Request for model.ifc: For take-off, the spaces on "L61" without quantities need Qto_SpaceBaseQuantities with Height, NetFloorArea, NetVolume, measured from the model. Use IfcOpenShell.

First a look at what the model holds.

```python
import ifcopenshell
import ifcopenshell.util.element
import ifcopenshell.util.unit

model = ifcopenshell.open("model.ifc")
print(model.schema)
for unit_type in ("LENGTHUNIT", "AREAUNIT", "VOLUMEUNIT"):
    print(unit_type, ifcopenshell.util.unit.calculate_unit_scale(model, unit_type))
storey = next(s for s in model.by_type("IfcBuildingStorey") if s.Name == "L61")
spaces = [e for e in ifcopenshell.util.element.get_decomposition(storey) if e.is_a("IfcSpace")]
for e in sorted(spaces, key=lambda e: e.id()):
    print(e.id(), e.is_a(), e.Name, list(ifcopenshell.util.element.get_psets(e, qtos_only=True)), sep=" | ")
```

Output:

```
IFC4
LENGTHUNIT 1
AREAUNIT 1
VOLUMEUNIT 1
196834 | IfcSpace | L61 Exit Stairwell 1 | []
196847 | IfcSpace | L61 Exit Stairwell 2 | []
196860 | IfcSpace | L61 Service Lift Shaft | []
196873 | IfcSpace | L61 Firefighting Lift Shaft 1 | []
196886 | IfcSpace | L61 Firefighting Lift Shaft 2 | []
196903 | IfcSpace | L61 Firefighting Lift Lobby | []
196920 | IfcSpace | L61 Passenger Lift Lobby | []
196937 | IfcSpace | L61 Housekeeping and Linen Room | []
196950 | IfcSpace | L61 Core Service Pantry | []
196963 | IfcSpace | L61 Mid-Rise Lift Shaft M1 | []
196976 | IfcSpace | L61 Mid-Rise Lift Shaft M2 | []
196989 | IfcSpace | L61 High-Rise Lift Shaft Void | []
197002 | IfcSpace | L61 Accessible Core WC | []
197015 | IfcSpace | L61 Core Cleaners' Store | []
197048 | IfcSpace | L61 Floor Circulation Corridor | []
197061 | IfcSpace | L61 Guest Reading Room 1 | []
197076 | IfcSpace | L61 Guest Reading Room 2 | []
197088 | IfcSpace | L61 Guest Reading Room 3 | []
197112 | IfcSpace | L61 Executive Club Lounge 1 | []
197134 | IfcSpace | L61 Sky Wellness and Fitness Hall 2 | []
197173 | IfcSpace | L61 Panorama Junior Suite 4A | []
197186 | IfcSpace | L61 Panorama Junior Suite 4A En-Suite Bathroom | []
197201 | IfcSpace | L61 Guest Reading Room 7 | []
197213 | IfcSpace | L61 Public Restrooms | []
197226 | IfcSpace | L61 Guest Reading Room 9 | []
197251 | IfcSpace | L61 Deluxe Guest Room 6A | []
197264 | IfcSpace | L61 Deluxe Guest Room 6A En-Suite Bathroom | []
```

```python
import ifcopenshell
import ifcopenshell.api.pset
import ifcopenshell.geom
import ifcopenshell.util.element
import ifcopenshell.util.shape
import ifcopenshell.util.unit

model = ifcopenshell.open("model.ifc")
unit_scale = ifcopenshell.util.unit.calculate_unit_scale(model)
area_scale = ifcopenshell.util.unit.calculate_unit_scale(model, "AREAUNIT")
volume_scale = ifcopenshell.util.unit.calculate_unit_scale(model, "VOLUMEUNIT")
settings = ifcopenshell.geom.settings()

storey = next(s for s in model.by_type("IfcBuildingStorey") if s.Name == "L61")
spaces = [e for e in ifcopenshell.util.element.get_decomposition(storey) if e.is_a("IfcSpace")]

for e in sorted(spaces, key=lambda e: e.id()):
    if ifcopenshell.util.element.get_psets(e, qtos_only=True, should_inherit=False):
        continue
    # Geometry comes back in metres, in the element's own axes.
    shape = ifcopenshell.geom.create_shape(settings, e)
    values = {
        "Height": ifcopenshell.util.shape.get_z(shape.geometry) / unit_scale,
        "NetFloorArea": ifcopenshell.util.shape.get_footprint_area(shape.geometry) / area_scale,
        "NetVolume": ifcopenshell.util.shape.get_volume(shape.geometry) / volume_scale,
    }
    qto = ifcopenshell.api.pset.add_qto(model, product=e, name="Qto_SpaceBaseQuantities")
    ifcopenshell.api.pset.edit_qto(model, qto=qto, properties=values)
    print(e.id(), {k: round(v, 3) for k, v in values.items()})

model.write("model_v2.ifc")
```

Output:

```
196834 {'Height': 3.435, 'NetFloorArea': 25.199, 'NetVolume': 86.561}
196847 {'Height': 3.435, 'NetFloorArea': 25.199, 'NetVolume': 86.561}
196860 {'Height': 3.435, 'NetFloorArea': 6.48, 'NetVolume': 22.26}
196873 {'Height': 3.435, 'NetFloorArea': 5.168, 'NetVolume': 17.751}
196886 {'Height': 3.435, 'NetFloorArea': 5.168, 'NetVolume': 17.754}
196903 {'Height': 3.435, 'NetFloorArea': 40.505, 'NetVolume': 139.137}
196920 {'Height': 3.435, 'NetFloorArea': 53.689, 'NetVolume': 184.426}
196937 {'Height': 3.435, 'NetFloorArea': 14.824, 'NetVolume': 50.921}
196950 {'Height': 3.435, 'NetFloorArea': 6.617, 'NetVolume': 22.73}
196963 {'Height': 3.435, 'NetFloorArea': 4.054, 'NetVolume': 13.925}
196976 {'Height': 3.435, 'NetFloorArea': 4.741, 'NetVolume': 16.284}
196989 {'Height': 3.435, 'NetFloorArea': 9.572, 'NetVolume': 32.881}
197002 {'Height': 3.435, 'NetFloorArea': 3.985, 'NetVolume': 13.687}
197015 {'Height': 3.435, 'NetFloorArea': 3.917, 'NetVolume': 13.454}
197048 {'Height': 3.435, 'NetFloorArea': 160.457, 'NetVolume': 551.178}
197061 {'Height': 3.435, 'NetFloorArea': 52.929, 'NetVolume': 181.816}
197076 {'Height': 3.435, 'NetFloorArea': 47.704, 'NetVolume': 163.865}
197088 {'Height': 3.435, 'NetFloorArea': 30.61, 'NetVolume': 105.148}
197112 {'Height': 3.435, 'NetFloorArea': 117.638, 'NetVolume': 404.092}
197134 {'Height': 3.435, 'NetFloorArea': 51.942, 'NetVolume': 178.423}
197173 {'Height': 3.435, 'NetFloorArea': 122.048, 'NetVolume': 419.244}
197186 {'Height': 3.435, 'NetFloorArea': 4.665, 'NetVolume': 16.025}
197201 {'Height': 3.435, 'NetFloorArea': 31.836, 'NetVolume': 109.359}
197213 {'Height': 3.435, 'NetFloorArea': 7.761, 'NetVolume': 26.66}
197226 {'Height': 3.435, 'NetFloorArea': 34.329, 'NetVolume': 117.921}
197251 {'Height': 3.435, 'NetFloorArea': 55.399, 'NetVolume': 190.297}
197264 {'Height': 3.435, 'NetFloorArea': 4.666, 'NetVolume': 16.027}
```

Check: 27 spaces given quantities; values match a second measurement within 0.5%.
